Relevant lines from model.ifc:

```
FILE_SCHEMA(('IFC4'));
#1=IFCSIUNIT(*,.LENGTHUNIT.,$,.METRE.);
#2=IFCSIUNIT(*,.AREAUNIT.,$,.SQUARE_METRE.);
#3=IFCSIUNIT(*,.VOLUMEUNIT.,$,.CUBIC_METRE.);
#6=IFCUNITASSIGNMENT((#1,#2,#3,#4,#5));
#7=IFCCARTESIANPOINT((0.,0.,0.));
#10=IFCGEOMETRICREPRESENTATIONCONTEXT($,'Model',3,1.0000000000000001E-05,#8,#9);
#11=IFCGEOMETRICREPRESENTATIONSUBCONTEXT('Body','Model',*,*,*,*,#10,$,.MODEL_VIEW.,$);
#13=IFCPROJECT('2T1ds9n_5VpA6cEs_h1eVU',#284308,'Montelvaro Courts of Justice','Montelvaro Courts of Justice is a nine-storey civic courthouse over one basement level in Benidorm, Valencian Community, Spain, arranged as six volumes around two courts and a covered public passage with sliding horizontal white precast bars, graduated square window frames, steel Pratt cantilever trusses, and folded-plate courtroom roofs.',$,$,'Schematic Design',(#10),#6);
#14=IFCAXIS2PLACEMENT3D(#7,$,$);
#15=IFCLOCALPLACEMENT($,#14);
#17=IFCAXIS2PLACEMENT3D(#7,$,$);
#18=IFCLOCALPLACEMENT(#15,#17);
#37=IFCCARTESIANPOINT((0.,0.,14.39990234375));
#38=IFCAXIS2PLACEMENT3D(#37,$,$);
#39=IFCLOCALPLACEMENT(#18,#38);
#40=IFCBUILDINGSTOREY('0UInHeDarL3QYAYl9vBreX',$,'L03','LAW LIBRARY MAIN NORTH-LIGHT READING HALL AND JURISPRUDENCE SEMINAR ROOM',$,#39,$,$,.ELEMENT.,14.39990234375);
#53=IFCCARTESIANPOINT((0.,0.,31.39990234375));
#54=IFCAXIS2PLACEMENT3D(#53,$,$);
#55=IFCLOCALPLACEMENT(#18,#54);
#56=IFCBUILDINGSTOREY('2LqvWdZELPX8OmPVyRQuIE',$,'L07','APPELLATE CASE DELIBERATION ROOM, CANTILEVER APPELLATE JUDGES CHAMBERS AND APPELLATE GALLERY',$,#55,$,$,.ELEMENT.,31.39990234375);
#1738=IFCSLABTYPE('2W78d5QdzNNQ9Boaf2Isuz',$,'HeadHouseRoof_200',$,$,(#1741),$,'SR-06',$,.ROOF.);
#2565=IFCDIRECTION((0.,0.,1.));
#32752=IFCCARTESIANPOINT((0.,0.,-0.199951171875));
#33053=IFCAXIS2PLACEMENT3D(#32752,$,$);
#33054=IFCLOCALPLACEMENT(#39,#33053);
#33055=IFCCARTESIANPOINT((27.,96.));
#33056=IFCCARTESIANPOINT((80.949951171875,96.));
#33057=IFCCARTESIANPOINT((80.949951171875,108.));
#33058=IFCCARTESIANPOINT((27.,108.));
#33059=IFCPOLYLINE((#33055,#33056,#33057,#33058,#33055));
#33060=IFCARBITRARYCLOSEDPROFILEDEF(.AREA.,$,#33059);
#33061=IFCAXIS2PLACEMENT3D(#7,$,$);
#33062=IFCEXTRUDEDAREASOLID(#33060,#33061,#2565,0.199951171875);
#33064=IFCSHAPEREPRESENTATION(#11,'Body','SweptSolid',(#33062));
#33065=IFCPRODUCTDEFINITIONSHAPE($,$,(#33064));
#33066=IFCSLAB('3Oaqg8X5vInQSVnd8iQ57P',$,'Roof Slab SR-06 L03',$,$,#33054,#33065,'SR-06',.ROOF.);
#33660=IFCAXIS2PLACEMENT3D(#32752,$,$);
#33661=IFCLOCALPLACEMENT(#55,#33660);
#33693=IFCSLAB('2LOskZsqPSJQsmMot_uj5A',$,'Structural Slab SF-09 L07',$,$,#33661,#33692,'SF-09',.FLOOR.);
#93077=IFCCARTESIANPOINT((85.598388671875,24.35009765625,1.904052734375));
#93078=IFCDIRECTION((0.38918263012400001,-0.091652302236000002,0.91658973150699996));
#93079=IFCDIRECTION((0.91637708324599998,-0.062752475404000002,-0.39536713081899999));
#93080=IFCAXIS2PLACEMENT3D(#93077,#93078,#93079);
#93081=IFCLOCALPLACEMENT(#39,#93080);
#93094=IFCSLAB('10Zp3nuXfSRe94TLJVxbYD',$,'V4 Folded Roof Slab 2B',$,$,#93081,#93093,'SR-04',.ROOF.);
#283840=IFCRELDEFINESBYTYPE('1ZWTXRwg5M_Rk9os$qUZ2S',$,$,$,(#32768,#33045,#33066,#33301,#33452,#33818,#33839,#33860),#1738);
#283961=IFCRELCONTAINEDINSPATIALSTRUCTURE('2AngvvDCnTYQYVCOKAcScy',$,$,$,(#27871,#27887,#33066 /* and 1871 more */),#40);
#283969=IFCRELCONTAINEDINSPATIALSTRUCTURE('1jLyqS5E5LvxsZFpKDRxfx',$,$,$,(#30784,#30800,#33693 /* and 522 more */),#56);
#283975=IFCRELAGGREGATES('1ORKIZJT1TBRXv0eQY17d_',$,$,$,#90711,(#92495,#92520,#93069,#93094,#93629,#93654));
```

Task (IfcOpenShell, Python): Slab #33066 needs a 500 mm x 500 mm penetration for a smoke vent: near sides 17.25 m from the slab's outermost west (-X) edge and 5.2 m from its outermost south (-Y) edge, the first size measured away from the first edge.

```python
import numpy as np
import ifcopenshell
import ifcopenshell.api.feature
import ifcopenshell.api.geometry
import ifcopenshell.api.root
import ifcopenshell.geom
import ifcopenshell.util.placement
import ifcopenshell.util.representation
import ifcopenshell.util.shape
import ifcopenshell.util.unit

model = ifcopenshell.open("model.ifc")
unit_scale = ifcopenshell.util.unit.calculate_unit_scale(model)
settings = ifcopenshell.geom.settings()


def volume(element):
    """Net volume in cubic metres, openings subtracted."""
    shape = ifcopenshell.geom.create_shape(settings, element)
    return ifcopenshell.util.shape.get_volume(shape.geometry)


slab = model.by_guid("3Oaqg8X5vInQSVnd8iQ57P")
before = volume(slab)

# Extent in the slab's own axes, in metres. The edges named are its -X and -Y sides.
slab_shape = ifcopenshell.geom.create_shape(settings, slab)
vertices = ifcopenshell.util.shape.get_vertices(slab_shape.geometry)
x_min, y_min, bottom = vertices.min(axis=0)
top = vertices[:, 2].max()

opening = ifcopenshell.api.root.create_entity(model, ifc_class="IfcOpeningElement", name="Smoke vent opening", predefined_type="OPENING")
context = ifcopenshell.util.representation.get_context(model, "Model", "Body", "MODEL_VIEW")
width, depth = 0.5, 0.5
outline = [(0.0, 0.0), (width, 0.0), (width, depth), (0.0, depth), (0.0, 0.0)]
# Overshoot both faces by 50 mm so the cut is clean.
shape = ifcopenshell.api.geometry.add_slab_representation(
    model, context=context, depth=top - bottom + 0.1, polyline=outline
)
ifcopenshell.api.geometry.assign_representation(model, product=opening, representation=shape)

matrix = ifcopenshell.util.placement.get_local_placement(slab.ObjectPlacement)
matrix[:, 3] = matrix @ np.append(np.array([x_min + 17.25, y_min + 5.2, bottom - 0.05]) / unit_scale, 1.0)
ifcopenshell.api.geometry.edit_object_placement(model, product=opening, matrix=matrix, is_si=False)
ifcopenshell.api.feature.add_feature(model, feature=opening, element=slab)

after = volume(slab)

print(f"slab volume {before:.3f} -> {after:.3f} m3")

model.write("model-out.ifc")
```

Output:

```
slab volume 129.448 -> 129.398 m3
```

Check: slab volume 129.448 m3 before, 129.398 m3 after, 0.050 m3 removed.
